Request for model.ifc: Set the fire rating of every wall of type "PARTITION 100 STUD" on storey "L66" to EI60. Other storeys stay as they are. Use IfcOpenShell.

First a look at what the model holds.

```python
import ifcopenshell
import ifcopenshell.util.element

model = ifcopenshell.open("model.ifc")
print(model.schema)
storey = next(s for s in model.by_type("IfcBuildingStorey") if s.Name == "L66")
walls = [e for e in ifcopenshell.util.element.get_decomposition(storey) if e.is_a("IfcWall")]
seen = {}
for e in walls:
    element_type = ifcopenshell.util.element.get_type(e)
    key = (element_type.Name if element_type != e and element_type else None, ifcopenshell.util.element.get_pset(e, "Pset_WallCommon", "FireRating"))
    seen[key] = seen.get(key, 0) + 1
for (name, value), count in sorted(seen.items(), key=str):
    print(count, "x", name, "|", value)
```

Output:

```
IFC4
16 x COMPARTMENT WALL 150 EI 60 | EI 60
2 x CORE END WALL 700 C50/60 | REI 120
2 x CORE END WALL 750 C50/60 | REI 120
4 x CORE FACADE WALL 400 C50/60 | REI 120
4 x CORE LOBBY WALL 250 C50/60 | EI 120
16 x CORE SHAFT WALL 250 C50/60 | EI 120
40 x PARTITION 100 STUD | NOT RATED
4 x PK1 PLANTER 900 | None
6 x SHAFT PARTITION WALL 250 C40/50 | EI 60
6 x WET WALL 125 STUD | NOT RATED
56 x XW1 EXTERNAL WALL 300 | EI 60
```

```python
import ifcopenshell
import ifcopenshell.api.pset
import ifcopenshell.util.element

model = ifcopenshell.open("model.ifc")

storey = next(s for s in model.by_type("IfcBuildingStorey") if s.Name == "L66")
walls = [e for e in ifcopenshell.util.element.get_decomposition(storey) if e.is_a("IfcWall")]

count = 0
for e in walls:
    element_type = ifcopenshell.util.element.get_type(e)
    if element_type in (None, e) or element_type.Name != "PARTITION 100 STUD":
        continue
    found = ifcopenshell.util.element.get_pset(e, "Pset_WallCommon", should_inherit=False)
    if found:
        pset = model.by_id(found["id"])
        if len(ifcopenshell.util.element.get_elements_by_pset(pset)) > 1:
            pset = ifcopenshell.api.pset.unshare_pset(model, products=[e], pset=pset)[0]
    else:
        pset = ifcopenshell.api.pset.add_pset(model, product=e, name="Pset_WallCommon")
    ifcopenshell.api.pset.edit_pset(model, pset=pset, properties={"FireRating": "EI60"})
    count += 1

print(count, "walls updated")

model.write("model_v2.ifc")
```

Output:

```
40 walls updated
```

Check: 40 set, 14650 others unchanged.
